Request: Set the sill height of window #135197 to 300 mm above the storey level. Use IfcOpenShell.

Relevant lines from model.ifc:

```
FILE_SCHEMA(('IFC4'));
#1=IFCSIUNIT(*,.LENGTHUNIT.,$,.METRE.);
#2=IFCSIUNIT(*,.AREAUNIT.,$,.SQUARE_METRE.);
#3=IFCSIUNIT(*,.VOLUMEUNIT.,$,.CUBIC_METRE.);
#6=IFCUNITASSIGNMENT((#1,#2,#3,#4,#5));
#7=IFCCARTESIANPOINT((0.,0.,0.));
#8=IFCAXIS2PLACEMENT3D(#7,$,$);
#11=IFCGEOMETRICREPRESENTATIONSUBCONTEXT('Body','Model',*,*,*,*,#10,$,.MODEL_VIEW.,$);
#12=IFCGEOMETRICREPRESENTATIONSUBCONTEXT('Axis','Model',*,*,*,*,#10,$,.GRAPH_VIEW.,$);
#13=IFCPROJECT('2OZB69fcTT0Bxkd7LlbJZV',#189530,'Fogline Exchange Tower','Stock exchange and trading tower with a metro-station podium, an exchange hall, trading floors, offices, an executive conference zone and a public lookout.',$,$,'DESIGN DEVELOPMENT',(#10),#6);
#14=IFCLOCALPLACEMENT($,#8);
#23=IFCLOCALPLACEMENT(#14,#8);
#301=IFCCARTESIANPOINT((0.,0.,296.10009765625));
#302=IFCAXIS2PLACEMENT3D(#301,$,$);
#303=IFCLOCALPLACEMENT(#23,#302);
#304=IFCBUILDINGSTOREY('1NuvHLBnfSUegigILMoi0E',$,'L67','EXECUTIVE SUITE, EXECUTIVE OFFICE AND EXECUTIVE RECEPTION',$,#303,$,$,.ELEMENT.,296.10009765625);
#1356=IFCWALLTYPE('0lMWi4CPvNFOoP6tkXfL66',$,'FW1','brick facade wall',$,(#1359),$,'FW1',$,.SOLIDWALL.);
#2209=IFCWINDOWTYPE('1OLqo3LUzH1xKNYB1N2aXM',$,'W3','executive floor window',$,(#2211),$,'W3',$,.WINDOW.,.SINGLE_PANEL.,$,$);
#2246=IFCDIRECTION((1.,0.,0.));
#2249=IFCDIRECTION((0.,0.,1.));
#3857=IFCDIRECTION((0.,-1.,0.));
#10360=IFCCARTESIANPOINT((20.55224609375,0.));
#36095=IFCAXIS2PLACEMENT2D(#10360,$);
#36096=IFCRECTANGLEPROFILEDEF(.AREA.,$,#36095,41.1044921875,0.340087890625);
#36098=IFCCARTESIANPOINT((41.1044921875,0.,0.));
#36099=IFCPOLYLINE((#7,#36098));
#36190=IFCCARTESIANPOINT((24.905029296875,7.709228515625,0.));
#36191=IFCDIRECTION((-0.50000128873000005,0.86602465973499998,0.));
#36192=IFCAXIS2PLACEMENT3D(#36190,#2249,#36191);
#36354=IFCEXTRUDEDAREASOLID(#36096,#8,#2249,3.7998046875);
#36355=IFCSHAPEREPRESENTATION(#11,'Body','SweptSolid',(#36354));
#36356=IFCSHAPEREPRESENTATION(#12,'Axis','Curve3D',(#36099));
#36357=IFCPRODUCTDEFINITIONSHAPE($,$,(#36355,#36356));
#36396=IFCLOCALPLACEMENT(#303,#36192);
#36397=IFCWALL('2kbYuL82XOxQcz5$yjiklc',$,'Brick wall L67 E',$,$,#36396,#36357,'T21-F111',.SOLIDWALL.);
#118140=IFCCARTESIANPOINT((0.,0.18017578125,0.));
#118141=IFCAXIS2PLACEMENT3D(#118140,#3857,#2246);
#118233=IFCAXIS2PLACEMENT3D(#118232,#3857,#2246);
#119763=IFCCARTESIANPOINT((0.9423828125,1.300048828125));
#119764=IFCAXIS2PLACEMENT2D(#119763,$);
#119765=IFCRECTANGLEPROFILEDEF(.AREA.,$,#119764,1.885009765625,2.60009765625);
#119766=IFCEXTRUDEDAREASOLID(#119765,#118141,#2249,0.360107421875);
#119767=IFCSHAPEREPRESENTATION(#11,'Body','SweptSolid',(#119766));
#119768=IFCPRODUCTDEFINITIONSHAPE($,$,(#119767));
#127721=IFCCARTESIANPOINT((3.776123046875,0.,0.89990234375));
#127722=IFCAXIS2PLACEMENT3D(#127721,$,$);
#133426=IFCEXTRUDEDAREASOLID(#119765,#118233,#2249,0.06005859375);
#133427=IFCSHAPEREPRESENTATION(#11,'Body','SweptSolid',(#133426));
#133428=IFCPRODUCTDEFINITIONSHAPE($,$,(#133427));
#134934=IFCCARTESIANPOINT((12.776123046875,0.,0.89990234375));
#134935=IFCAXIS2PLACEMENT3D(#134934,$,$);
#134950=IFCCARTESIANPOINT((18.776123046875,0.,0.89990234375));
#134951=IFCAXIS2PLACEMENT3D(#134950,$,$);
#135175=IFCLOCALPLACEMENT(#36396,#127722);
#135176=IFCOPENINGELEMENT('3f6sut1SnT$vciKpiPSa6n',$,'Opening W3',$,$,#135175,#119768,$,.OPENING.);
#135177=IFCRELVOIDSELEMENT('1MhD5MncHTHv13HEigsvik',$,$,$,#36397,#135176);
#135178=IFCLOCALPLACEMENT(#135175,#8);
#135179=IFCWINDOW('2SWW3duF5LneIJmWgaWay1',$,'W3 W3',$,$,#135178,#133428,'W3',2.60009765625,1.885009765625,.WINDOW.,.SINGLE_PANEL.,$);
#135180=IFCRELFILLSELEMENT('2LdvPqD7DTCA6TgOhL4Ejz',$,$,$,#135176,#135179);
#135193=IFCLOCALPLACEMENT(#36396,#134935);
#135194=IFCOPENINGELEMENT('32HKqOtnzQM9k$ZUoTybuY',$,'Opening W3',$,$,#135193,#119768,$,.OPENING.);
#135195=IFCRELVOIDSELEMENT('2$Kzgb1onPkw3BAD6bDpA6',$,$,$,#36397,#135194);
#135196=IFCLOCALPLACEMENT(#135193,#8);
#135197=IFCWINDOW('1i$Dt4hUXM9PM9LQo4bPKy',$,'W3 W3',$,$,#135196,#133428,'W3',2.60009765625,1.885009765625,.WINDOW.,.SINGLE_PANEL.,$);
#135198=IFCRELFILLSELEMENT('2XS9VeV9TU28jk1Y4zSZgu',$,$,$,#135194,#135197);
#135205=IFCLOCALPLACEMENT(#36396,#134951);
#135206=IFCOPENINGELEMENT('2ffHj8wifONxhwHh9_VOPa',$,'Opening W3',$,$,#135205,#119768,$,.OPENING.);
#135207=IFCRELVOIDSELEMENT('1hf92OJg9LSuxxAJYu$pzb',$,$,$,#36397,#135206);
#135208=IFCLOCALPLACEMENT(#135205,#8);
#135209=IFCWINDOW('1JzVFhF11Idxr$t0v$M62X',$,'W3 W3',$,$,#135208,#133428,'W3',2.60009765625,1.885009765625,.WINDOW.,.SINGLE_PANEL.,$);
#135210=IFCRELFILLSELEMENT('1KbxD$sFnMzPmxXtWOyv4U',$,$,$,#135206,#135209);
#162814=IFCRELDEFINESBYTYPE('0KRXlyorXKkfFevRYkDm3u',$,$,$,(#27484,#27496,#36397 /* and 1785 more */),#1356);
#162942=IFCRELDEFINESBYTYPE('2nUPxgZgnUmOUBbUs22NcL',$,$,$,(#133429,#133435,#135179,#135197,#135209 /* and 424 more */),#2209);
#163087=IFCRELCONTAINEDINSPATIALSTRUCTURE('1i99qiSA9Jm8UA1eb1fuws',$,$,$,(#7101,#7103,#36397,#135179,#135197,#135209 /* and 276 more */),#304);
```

```python
import numpy as np
import ifcopenshell
import ifcopenshell.api.geometry
import ifcopenshell.geom
import ifcopenshell.util.element
import ifcopenshell.util.placement
import ifcopenshell.util.shape
import ifcopenshell.util.unit

model = ifcopenshell.open("model.ifc")
unit_scale = ifcopenshell.util.unit.calculate_unit_scale(model)

window = model.by_guid("1i$Dt4hUXM9PM9LQo4bPKy")
opening = window.FillsVoids[0].RelatingOpeningElement
storey = ifcopenshell.util.element.get_container(window, ifc_class="IfcBuildingStorey")
level = ifcopenshell.util.placement.get_local_placement(storey.ObjectPlacement)[2, 3]

# The opening's origin need not be at the sill, so measure its lowest point.
shape = ifcopenshell.geom.create_shape(ifcopenshell.geom.settings(), opening)
bottom = ifcopenshell.util.shape.get_shape_bottom_elevation(shape, shape.geometry) / unit_scale
dz = level + 0.3 / unit_scale - bottom

shift = np.array([0.0, 0.0, dz])
# The window is placed relative to its opening, so it follows when the opening moves.
matrix = ifcopenshell.util.placement.get_local_placement(opening.ObjectPlacement)
matrix[:3, 3] += shift
ifcopenshell.api.geometry.edit_object_placement(
    model, product=opening, matrix=matrix, is_si=False, should_transform_children=True
)

print(f"moved by {dz * unit_scale:+.3f} m")

model.write("model_updated.ifc")
```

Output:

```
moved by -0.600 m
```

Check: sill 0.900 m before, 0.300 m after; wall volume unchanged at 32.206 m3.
